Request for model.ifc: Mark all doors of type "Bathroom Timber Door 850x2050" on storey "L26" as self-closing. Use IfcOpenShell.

First a look at what the model holds.

```python
import ifcopenshell
import ifcopenshell.util.element

model = ifcopenshell.open("model.ifc")
print(model.schema)
storey = next(s for s in model.by_type("IfcBuildingStorey") if s.Name == "L26")
doors = [e for e in ifcopenshell.util.element.get_decomposition(storey) if e.is_a("IfcDoor")]
seen = {}
for e in doors:
    element_type = ifcopenshell.util.element.get_type(e)
    key = (element_type.Name if element_type != e and element_type else None, ifcopenshell.util.element.get_pset(e, "Pset_DoorCommon", "SelfClosing"))
    seen[key] = seen.get(key, 0) + 1
for (name, value), count in sorted(seen.items(), key=str):
    print(count, "x", name, "|", value)
```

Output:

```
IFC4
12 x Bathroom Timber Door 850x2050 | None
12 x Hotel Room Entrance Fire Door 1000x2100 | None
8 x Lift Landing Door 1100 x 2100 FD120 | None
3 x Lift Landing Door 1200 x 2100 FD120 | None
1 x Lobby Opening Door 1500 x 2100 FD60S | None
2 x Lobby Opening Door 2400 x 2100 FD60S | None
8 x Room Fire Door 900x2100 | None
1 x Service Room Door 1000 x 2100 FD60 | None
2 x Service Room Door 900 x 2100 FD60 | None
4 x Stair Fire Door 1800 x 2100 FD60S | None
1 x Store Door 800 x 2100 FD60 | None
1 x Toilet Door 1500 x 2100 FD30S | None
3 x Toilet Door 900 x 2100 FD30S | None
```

```python
import ifcopenshell
import ifcopenshell.api.pset
import ifcopenshell.util.element

model = ifcopenshell.open("model.ifc")

storey = next(s for s in model.by_type("IfcBuildingStorey") if s.Name == "L26")
doors = [e for e in ifcopenshell.util.element.get_decomposition(storey) if e.is_a("IfcDoor")]

count = 0
for e in doors:
    element_type = ifcopenshell.util.element.get_type(e)
    if element_type in (None, e) or element_type.Name != "Bathroom Timber Door 850x2050":
        continue
    found = ifcopenshell.util.element.get_pset(e, "Pset_DoorCommon", should_inherit=False)
    if found:
        pset = model.by_id(found["id"])
        if len(ifcopenshell.util.element.get_elements_by_pset(pset)) > 1:
            pset = ifcopenshell.api.pset.unshare_pset(model, products=[e], pset=pset)[0]
    else:
        pset = ifcopenshell.api.pset.add_pset(model, product=e, name="Pset_DoorCommon")
    ifcopenshell.api.pset.edit_pset(model, pset=pset, properties={"SelfClosing": True})
    count += 1

print(count, "doors updated")

model.write("model_v2.ifc")
```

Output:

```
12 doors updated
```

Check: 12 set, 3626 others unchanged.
